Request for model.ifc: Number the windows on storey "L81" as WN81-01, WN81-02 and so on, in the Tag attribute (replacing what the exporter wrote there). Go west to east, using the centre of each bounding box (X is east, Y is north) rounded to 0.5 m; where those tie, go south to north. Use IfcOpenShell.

First a look at what the model holds.

```python
import ifcopenshell
import ifcopenshell.util.element
import ifcopenshell.util.placement

model = ifcopenshell.open("model.ifc")
print(model.schema)
storey = next(s for s in model.by_type("IfcBuildingStorey") if s.Name == "L81")
windows = [e for e in ifcopenshell.util.element.get_decomposition(storey) if e.is_a("IfcWindow")]
for e in sorted(windows, key=lambda e: e.id()):
    origin = ifcopenshell.util.placement.get_local_placement(e.ObjectPlacement)[:3, 3]
    print(e.id(), e.Tag, e.Name, origin.round(2) + 0.0, sep=" | ")
```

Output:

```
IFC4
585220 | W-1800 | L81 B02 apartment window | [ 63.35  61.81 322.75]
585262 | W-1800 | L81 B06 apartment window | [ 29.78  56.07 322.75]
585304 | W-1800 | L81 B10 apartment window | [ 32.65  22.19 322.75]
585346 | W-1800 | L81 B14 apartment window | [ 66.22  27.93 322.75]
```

```python
import ifcopenshell
import ifcopenshell.geom
import ifcopenshell.util.element
import ifcopenshell.util.shape

model = ifcopenshell.open("model.ifc")
settings = ifcopenshell.geom.settings()
settings.set("use-world-coords", True)


def centre(element):
    shape = ifcopenshell.geom.create_shape(settings, element)
    return ifcopenshell.util.shape.get_bbox_centroid(shape.geometry)


storey = next(s for s in model.by_type("IfcBuildingStorey") if s.Name == "L81")
windows = [e for e in ifcopenshell.util.element.get_decomposition(storey) if e.is_a("IfcWindow")]

# Insertion points can sit at a corner or the storey origin, so sort by the geometry (in metres).
centres = {e: centre(e) for e in windows}
windows.sort(key=lambda e: (round(centres[e][0] / 0.5), centres[e][1]))

for i, e in enumerate(windows, start=1):
    number = f"WN81-{i:02d}"
    e.Tag = number
    print(e.id(), number)

model.write("model_v2.ifc")
```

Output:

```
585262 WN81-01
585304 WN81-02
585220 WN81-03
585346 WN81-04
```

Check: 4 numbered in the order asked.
